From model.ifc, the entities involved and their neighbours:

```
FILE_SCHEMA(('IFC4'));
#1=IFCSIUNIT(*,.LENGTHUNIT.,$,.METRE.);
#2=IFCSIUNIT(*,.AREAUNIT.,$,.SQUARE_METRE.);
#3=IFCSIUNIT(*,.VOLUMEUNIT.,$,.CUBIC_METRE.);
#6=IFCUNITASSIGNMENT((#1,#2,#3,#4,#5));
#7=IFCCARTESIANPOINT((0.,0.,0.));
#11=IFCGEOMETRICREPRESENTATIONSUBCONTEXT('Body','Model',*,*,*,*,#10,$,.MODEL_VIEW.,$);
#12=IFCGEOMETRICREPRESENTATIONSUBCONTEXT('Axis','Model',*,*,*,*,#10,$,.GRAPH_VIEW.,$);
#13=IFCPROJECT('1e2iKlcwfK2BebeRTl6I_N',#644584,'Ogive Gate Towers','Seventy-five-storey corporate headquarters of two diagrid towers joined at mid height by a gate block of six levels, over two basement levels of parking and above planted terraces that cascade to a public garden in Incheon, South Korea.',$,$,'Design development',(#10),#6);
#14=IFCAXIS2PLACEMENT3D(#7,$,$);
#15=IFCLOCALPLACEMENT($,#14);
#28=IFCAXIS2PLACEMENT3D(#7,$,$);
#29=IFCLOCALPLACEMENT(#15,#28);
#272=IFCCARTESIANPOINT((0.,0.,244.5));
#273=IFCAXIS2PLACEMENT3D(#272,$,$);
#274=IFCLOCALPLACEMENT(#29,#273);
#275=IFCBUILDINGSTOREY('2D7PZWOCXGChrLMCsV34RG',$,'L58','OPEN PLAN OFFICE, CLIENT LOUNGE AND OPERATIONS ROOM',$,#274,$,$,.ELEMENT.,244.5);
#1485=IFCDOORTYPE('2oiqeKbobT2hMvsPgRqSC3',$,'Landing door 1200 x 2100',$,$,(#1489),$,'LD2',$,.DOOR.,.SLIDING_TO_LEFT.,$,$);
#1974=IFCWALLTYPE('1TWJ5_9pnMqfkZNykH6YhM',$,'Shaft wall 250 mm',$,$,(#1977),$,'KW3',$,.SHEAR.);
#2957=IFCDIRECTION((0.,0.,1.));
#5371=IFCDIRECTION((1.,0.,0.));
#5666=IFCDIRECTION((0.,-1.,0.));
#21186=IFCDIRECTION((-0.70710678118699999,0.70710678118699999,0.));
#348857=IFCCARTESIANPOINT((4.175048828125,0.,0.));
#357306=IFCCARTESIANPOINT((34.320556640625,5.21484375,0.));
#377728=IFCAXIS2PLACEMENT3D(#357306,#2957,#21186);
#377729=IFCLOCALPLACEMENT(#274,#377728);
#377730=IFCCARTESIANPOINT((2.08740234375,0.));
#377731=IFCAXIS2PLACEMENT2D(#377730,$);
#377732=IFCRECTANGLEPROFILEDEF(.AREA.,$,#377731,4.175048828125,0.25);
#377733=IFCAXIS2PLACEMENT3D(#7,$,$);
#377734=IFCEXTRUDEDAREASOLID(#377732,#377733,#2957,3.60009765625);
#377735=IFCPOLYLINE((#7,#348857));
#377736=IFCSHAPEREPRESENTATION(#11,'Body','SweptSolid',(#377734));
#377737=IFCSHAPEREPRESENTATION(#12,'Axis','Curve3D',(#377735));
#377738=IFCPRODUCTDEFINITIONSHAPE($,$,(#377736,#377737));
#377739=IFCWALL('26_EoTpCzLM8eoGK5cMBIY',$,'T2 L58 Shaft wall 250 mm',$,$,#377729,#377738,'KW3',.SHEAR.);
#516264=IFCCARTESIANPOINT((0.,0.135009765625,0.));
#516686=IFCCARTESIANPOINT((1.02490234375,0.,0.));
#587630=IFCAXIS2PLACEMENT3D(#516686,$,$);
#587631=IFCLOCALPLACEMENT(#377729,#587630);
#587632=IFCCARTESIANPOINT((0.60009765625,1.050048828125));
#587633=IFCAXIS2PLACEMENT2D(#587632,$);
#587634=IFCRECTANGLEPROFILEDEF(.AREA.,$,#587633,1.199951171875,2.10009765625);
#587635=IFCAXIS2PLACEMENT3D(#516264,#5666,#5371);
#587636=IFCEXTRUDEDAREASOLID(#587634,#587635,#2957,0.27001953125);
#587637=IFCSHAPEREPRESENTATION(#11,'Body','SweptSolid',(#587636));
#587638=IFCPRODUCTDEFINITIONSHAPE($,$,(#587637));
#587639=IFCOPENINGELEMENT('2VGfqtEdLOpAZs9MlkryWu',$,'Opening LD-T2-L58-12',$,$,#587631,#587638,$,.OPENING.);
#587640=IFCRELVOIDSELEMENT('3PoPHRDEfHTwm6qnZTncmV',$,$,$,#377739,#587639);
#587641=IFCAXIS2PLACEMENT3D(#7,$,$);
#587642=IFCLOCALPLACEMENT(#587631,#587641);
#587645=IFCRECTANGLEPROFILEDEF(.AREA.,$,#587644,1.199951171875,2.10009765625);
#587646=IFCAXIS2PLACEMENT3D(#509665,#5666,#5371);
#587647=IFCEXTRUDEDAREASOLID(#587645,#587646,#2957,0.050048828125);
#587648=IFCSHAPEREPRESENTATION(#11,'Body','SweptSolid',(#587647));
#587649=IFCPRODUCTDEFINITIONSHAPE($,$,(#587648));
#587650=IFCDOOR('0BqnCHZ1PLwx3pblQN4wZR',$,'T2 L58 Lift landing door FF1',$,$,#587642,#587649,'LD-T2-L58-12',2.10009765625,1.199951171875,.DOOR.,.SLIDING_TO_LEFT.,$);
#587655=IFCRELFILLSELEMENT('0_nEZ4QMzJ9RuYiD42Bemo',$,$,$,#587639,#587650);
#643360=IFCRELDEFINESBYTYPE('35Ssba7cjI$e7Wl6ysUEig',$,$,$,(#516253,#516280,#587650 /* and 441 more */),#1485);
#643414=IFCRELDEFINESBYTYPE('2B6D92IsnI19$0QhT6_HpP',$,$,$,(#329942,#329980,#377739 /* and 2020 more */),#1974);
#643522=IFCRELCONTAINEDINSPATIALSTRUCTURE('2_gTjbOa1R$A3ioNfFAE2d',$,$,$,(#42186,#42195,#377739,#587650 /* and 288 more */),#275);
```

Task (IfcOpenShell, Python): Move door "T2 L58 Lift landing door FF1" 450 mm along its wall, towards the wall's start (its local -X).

```python
import ifcopenshell
import ifcopenshell.api.geometry
import ifcopenshell.util.placement
import ifcopenshell.util.unit

model = ifcopenshell.open("model.ifc")
unit_scale = ifcopenshell.util.unit.calculate_unit_scale(model)

door = model.by_guid("0BqnCHZ1PLwx3pblQN4wZR")
opening = door.FillsVoids[0].RelatingOpeningElement
wall = opening.VoidsElements[0].RelatingBuildingElement

wall_matrix = ifcopenshell.util.placement.get_local_placement(wall.ObjectPlacement)
shift = wall_matrix[:3, 0] * -0.45 / unit_scale
before = ifcopenshell.util.placement.get_local_placement(door.ObjectPlacement)[:3, 3].copy()

# The door is placed relative to its opening, so it follows when the opening moves.
matrix = ifcopenshell.util.placement.get_local_placement(opening.ObjectPlacement)
matrix[:3, 3] += shift
ifcopenshell.api.geometry.edit_object_placement(
    model, product=opening, matrix=matrix, is_si=False, should_transform_children=True
)

after = ifcopenshell.util.placement.get_local_placement(door.ObjectPlacement)[:3, 3]
print("door moved by", (after - before).round(3) + 0.0)

model.write("model_v2.ifc")
```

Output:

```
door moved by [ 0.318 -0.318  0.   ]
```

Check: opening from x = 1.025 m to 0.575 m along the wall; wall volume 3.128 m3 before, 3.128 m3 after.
